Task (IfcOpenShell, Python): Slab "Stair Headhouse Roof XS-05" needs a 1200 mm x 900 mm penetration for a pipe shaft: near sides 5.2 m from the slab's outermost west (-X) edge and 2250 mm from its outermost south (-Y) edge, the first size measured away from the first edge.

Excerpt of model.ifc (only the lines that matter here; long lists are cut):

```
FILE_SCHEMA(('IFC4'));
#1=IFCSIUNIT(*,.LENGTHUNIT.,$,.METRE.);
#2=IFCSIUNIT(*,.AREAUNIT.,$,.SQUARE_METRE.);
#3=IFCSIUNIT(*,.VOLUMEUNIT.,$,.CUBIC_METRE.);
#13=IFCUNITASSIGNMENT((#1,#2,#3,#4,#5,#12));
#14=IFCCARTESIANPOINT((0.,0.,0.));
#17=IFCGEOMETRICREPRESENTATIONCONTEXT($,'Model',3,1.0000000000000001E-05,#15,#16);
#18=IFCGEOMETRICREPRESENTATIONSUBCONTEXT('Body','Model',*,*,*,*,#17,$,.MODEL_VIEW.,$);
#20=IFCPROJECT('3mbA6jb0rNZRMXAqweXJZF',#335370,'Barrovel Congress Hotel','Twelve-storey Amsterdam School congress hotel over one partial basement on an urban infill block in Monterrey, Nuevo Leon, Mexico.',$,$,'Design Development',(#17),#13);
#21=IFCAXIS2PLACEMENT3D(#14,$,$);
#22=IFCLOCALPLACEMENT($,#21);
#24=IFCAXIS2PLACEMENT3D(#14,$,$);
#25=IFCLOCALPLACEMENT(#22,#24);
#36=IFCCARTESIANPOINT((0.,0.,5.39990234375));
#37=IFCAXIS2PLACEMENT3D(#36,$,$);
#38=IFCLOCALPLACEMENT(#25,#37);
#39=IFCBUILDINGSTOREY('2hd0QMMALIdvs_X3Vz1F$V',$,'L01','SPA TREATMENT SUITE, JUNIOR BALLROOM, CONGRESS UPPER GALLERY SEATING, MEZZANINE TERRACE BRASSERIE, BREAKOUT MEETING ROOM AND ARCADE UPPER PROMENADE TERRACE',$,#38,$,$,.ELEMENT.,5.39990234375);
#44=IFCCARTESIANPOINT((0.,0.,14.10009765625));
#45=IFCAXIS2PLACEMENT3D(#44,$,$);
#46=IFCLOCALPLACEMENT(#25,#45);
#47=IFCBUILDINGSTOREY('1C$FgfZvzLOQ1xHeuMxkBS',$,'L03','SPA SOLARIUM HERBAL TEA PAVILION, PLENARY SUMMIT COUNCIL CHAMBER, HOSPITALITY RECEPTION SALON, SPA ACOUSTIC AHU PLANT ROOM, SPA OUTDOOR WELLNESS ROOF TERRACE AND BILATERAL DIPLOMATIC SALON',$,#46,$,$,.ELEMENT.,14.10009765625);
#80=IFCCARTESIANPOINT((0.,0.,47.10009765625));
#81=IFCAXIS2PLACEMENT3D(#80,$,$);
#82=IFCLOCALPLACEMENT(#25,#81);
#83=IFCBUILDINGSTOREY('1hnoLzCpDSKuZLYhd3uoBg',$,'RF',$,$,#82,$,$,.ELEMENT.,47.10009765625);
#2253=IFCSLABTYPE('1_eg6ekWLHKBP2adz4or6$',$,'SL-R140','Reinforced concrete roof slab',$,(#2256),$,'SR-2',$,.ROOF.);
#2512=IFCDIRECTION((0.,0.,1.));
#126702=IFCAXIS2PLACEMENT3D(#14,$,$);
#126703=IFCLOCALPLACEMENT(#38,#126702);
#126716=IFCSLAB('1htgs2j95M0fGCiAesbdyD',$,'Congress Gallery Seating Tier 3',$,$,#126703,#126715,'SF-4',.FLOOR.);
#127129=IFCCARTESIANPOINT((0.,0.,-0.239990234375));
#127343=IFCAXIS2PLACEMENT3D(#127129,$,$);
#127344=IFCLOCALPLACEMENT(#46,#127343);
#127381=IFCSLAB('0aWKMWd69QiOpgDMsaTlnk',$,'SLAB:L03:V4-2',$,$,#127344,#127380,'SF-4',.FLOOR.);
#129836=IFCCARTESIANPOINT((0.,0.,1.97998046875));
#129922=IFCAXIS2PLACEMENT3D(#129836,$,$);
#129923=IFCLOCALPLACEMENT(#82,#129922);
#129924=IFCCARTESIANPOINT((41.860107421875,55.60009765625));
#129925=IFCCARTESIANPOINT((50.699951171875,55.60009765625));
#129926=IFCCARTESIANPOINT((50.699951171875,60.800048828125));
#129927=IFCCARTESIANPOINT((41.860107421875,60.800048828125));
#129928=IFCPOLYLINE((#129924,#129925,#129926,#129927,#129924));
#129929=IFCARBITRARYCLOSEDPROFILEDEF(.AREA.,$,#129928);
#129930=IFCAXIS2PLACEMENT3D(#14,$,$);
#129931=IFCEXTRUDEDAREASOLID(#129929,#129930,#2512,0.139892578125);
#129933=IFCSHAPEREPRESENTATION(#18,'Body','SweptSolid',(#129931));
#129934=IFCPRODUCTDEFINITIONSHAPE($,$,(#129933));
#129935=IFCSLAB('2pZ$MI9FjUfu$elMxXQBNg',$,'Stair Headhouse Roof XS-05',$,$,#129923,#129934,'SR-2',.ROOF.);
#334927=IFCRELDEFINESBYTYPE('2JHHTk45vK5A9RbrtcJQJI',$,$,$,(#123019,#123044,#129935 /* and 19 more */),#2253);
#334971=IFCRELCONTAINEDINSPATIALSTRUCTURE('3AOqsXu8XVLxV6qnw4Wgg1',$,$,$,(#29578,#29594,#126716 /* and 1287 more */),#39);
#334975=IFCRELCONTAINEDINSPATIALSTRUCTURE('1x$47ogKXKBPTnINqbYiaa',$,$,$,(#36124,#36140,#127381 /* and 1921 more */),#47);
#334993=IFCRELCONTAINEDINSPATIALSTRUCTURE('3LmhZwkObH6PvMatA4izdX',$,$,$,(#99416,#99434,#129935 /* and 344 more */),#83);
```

```python
import numpy as np
import ifcopenshell
import ifcopenshell.api.feature
import ifcopenshell.api.geometry
import ifcopenshell.api.root
import ifcopenshell.geom
import ifcopenshell.util.placement
import ifcopenshell.util.representation
import ifcopenshell.util.shape
import ifcopenshell.util.unit

model = ifcopenshell.open("model.ifc")
unit_scale = ifcopenshell.util.unit.calculate_unit_scale(model)
settings = ifcopenshell.geom.settings()


def volume(element):
    """Net volume in cubic metres, openings subtracted."""
    shape = ifcopenshell.geom.create_shape(settings, element)
    return ifcopenshell.util.shape.get_volume(shape.geometry)


slab = model.by_guid("2pZ$MI9FjUfu$elMxXQBNg")
before = volume(slab)

# Extent in the slab's own axes, in metres. The edges named are its -X and -Y sides.
slab_shape = ifcopenshell.geom.create_shape(settings, slab)
vertices = ifcopenshell.util.shape.get_vertices(slab_shape.geometry)
x_min, y_min, bottom = vertices.min(axis=0)
top = vertices[:, 2].max()

opening = ifcopenshell.api.root.create_entity(model, ifc_class="IfcOpeningElement", name="Pipe shaft opening", predefined_type="OPENING")
context = ifcopenshell.util.representation.get_context(model, "Model", "Body", "MODEL_VIEW")
width, depth = 1.2, 0.9
outline = [(0.0, 0.0), (width, 0.0), (width, depth), (0.0, depth), (0.0, 0.0)]
# Overshoot both faces by 50 mm so the cut is clean.
shape = ifcopenshell.api.geometry.add_slab_representation(
    model, context=context, depth=top - bottom + 0.1, polyline=outline
)
ifcopenshell.api.geometry.assign_representation(model, product=opening, representation=shape)

matrix = ifcopenshell.util.placement.get_local_placement(slab.ObjectPlacement)
matrix[:, 3] = matrix @ np.append(np.array([x_min + 5.2, y_min + 2.25, bottom - 0.05]) / unit_scale, 1.0)
ifcopenshell.api.geometry.edit_object_placement(model, product=opening, matrix=matrix, is_si=False)
ifcopenshell.api.feature.add_feature(model, feature=opening, element=slab)

after = volume(slab)

print(f"slab volume {before:.3f} -> {after:.3f} m3")

model.write("model_rev.ifc")
```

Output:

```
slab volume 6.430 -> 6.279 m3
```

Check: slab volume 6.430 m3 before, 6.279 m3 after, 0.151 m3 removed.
